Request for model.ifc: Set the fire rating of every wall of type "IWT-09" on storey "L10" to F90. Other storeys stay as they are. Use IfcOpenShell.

First a look at what the model holds.

```python
import ifcopenshell
import ifcopenshell.util.element

model = ifcopenshell.open("model.ifc")
print(model.schema)
storey = next(s for s in model.by_type("IfcBuildingStorey") if s.Name == "L10")
walls = [e for e in ifcopenshell.util.element.get_decomposition(storey) if e.is_a("IfcWall")]
seen = {}
for e in walls:
    element_type = ifcopenshell.util.element.get_type(e)
    key = (element_type.Name if element_type != e and element_type else None, ifcopenshell.util.element.get_pset(e, "Pset_WallCommon", "FireRating"))
    seen[key] = seen.get(key, 0) + 1
for (name, value), count in sorted(seen.items(), key=str):
    print(count, "x", name, "|", value)
```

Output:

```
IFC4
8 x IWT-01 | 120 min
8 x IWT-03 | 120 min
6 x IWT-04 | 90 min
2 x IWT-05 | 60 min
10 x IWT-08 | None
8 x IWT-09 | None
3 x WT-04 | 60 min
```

```python
import ifcopenshell
import ifcopenshell.api.pset
import ifcopenshell.util.element

model = ifcopenshell.open("model.ifc")

storey = next(s for s in model.by_type("IfcBuildingStorey") if s.Name == "L10")
walls = [e for e in ifcopenshell.util.element.get_decomposition(storey) if e.is_a("IfcWall")]

count = 0
for e in walls:
    element_type = ifcopenshell.util.element.get_type(e)
    if element_type in (None, e) or element_type.Name != "IWT-09":
        continue
    # add_pset returns the element's existing set when there is one.
    pset = ifcopenshell.api.pset.add_pset(model, product=e, name="Pset_WallCommon")
    ifcopenshell.api.pset.edit_pset(model, pset=pset, properties={"FireRating": "F90"})
    count += 1

print(count, "walls updated")

model.write("model_rev.ifc")
```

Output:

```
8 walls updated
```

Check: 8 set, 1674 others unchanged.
